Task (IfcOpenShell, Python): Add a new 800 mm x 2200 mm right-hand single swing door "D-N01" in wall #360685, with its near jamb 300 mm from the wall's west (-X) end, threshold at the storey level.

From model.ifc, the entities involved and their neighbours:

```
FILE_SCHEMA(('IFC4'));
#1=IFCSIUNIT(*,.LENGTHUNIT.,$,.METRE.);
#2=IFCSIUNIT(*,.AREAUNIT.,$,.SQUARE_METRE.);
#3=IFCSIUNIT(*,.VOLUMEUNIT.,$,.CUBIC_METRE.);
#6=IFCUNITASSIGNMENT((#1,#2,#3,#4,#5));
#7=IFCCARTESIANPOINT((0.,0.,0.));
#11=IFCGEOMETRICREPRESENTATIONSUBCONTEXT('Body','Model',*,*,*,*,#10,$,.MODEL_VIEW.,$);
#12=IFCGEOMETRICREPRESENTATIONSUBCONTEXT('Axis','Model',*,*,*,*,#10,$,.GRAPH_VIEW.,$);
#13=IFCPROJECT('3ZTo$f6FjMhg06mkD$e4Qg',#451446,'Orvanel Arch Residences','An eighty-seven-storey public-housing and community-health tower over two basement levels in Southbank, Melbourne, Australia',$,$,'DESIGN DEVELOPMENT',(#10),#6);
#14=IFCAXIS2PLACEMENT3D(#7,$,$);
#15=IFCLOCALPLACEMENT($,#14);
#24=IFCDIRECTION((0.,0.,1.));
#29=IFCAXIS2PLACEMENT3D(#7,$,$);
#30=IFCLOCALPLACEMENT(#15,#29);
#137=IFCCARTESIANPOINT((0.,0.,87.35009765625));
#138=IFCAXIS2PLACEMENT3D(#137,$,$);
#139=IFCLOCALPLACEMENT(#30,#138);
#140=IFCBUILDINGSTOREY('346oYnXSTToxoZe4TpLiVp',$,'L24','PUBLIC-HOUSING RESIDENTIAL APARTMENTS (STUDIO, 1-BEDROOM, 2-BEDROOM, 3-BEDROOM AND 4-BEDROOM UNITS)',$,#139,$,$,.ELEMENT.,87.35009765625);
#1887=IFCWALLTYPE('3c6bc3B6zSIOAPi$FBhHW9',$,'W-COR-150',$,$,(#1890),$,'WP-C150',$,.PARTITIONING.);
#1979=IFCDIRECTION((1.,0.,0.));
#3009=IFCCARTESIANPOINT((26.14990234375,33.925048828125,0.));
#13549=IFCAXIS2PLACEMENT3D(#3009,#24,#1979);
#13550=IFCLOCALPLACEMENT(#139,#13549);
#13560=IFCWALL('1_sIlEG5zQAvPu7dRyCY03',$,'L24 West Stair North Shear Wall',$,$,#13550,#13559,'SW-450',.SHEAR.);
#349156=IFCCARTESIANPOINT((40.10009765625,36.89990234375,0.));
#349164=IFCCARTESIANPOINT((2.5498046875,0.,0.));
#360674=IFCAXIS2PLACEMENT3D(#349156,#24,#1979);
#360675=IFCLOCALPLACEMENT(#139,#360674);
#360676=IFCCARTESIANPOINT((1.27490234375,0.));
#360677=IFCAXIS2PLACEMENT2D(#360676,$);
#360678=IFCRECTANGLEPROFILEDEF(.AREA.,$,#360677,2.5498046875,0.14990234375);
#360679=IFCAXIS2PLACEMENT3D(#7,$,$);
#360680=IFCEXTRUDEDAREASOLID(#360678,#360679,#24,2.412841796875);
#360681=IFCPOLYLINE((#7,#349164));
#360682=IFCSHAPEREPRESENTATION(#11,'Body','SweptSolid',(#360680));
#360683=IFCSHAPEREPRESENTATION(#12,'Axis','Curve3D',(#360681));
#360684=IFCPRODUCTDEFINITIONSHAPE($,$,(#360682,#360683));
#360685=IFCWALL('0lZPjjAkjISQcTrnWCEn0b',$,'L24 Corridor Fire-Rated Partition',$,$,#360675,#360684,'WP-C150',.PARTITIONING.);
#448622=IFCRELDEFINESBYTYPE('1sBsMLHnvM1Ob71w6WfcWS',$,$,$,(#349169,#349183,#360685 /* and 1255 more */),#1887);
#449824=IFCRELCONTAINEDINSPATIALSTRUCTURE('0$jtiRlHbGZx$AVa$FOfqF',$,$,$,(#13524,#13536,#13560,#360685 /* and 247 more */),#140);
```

```python
import numpy as np
import ifcopenshell
import ifcopenshell.api.feature
import ifcopenshell.api.geometry
import ifcopenshell.api.root
import ifcopenshell.api.spatial
import ifcopenshell.geom
import ifcopenshell.util.element
import ifcopenshell.util.placement
import ifcopenshell.util.representation
import ifcopenshell.util.shape
import ifcopenshell.util.unit

model = ifcopenshell.open("model.ifc")
unit_scale = ifcopenshell.util.unit.calculate_unit_scale(model)
settings = ifcopenshell.geom.settings()


def volume(element):
    """Net volume in cubic metres, openings subtracted."""
    shape = ifcopenshell.geom.create_shape(settings, element)
    return ifcopenshell.util.shape.get_volume(shape.geometry)


wall = model.by_id(360685)
storey = ifcopenshell.util.element.get_container(wall, ifc_class="IfcBuildingStorey")
context = ifcopenshell.util.representation.get_context(model, "Model", "Body", "MODEL_VIEW")
before = volume(wall)

width, height, from_end, sill = 0.8, 2.2, 0.3, 0.0  # metres

# The wall runs along its own X axis, and the end named is its -X end.
wall_shape = ifcopenshell.geom.create_shape(settings, wall)
x, y, z = ifcopenshell.util.shape.get_vertices(wall_shape.geometry).T
start = x.min() + from_end
face, thickness = float(y.min()), float(y.max() - y.min())
wall_matrix = ifcopenshell.util.placement.get_local_placement(wall.ObjectPlacement)
level = ifcopenshell.util.placement.get_local_placement(storey.ObjectPlacement)[2, 3]


def in_wall(x, y):
    """Placement at x, y metres in the wall's axes, at sill height."""
    matrix = wall_matrix.copy()
    matrix[:, 3] = wall_matrix @ np.array([x / unit_scale, y / unit_scale, 0.0, 1.0])
    matrix[2, 3] = level + sill / unit_scale
    return matrix


# Opening: a box that overshoots both wall faces by 50 mm.
opening = ifcopenshell.api.root.create_entity(model, ifc_class="IfcOpeningElement", predefined_type="OPENING")
box = ifcopenshell.api.geometry.add_wall_representation(
    model, context=context, length=width, height=height, thickness=thickness + 0.1
)
ifcopenshell.api.geometry.assign_representation(model, product=opening, representation=box)
ifcopenshell.api.geometry.edit_object_placement(model, product=opening, matrix=in_wall(start, face - 0.05), is_si=False)
ifcopenshell.api.feature.add_feature(model, feature=opening, element=wall)

door = ifcopenshell.api.root.create_entity(model, ifc_class="IfcDoor", name="D-N01", predefined_type="DOOR")
door.OverallWidth, door.OverallHeight = width / unit_scale, height / unit_scale
door.OperationType = "SINGLE_SWING_RIGHT"
body = ifcopenshell.api.geometry.add_door_representation(
    model,
    context=context,
    overall_width=door.OverallWidth,
    overall_height=door.OverallHeight,
    operation_type="SINGLE_SWING_RIGHT",
    lining_properties={"LiningDepth": thickness / unit_scale, "ThresholdDepth": thickness / unit_scale},
)
ifcopenshell.api.geometry.assign_representation(model, product=door, representation=body)
ifcopenshell.api.spatial.assign_container(model, products=[door], relating_structure=storey)
ifcopenshell.api.feature.add_filling(model, opening=opening, element=door)

# The lining spans the wall, so the door starts at the wall face.
ifcopenshell.api.geometry.edit_object_placement(model, product=door, matrix=in_wall(start, face), is_si=False)

after = volume(wall)

print(f"wall volume {before:.3f} -> {after:.3f} m3")

model.write("model_rev.ifc")
```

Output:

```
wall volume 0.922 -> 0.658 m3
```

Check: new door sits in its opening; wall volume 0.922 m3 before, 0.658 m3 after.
